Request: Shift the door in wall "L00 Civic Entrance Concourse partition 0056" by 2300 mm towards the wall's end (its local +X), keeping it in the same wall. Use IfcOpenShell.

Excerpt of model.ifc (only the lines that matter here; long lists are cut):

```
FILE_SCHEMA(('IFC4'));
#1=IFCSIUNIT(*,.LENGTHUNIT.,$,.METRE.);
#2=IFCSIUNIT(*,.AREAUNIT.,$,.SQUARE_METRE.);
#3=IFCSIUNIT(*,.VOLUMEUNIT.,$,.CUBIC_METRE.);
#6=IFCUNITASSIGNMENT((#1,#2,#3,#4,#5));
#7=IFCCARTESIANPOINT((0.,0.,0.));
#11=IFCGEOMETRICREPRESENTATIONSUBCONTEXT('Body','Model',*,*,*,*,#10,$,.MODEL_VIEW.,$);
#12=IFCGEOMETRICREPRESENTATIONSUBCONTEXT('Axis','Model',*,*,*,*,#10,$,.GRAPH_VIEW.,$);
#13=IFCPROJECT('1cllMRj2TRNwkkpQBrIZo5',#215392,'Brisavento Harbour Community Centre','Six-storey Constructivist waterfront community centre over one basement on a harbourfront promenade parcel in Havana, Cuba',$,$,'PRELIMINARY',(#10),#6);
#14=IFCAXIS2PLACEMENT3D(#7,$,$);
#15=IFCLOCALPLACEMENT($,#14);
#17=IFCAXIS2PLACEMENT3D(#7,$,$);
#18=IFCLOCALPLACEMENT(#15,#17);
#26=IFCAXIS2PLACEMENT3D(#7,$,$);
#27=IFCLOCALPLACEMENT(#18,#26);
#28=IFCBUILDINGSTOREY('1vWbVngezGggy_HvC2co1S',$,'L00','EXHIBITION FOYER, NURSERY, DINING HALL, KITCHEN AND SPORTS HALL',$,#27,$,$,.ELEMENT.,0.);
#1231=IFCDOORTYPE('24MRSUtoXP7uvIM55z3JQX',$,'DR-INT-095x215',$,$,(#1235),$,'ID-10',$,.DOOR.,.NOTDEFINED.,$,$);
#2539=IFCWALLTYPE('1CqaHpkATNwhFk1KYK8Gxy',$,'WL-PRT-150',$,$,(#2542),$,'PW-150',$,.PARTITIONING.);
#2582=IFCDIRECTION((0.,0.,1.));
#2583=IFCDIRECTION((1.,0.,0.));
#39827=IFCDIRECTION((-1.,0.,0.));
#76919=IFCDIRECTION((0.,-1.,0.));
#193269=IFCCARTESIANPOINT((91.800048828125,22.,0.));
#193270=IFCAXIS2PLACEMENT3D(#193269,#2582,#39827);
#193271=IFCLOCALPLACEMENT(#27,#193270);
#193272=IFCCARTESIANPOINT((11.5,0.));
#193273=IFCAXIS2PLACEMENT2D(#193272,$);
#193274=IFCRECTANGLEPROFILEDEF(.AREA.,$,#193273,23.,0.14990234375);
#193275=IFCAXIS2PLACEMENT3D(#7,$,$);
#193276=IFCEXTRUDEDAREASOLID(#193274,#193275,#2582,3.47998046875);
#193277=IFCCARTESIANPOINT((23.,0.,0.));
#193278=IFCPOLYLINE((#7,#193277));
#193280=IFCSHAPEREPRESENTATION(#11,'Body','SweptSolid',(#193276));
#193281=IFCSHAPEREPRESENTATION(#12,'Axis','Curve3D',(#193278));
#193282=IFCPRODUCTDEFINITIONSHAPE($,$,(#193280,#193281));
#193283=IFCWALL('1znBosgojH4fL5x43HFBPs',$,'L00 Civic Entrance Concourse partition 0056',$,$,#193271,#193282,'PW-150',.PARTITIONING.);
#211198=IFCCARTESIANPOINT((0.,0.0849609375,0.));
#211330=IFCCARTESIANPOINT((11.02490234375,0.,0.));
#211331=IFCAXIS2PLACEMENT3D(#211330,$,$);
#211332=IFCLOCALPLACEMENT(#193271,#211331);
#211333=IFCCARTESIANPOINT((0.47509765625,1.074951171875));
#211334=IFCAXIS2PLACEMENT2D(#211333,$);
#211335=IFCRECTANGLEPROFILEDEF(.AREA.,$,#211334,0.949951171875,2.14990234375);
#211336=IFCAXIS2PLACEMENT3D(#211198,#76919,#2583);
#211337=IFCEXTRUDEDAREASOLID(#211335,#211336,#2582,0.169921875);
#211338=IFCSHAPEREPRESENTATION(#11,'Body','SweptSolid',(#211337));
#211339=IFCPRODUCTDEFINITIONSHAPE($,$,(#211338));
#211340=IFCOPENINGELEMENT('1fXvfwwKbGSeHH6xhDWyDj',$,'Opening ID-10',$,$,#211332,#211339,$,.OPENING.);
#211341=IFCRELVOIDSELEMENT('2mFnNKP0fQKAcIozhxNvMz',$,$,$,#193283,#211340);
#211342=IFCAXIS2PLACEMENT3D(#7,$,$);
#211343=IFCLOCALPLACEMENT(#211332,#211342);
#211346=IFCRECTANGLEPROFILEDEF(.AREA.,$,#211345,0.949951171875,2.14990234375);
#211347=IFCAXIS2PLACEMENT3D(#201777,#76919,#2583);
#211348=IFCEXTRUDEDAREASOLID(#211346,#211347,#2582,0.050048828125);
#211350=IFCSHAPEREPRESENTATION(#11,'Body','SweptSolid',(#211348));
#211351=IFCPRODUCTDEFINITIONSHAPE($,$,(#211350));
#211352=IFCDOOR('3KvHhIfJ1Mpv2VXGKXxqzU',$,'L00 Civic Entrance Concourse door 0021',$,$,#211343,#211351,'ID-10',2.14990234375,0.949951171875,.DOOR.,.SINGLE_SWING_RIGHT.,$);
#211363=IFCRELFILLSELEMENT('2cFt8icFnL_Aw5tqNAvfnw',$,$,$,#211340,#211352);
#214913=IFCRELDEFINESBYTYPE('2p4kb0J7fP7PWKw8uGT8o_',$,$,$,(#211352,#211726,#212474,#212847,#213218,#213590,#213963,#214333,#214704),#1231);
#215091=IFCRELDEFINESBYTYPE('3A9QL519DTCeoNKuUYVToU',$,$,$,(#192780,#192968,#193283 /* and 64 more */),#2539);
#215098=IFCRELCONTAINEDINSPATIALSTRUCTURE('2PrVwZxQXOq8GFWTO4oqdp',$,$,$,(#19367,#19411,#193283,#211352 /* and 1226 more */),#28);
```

```python
import ifcopenshell
import ifcopenshell.api.geometry
import ifcopenshell.util.placement
import ifcopenshell.util.unit

model = ifcopenshell.open("model.ifc")
unit_scale = ifcopenshell.util.unit.calculate_unit_scale(model)

door = model.by_id(211352)
opening = door.FillsVoids[0].RelatingOpeningElement
wall = opening.VoidsElements[0].RelatingBuildingElement

wall_matrix = ifcopenshell.util.placement.get_local_placement(wall.ObjectPlacement)
shift = wall_matrix[:3, 0] * 2.3 / unit_scale
before = ifcopenshell.util.placement.get_local_placement(door.ObjectPlacement)[:3, 3].copy()

# The door is placed relative to its opening, so it follows when the opening moves.
matrix = ifcopenshell.util.placement.get_local_placement(opening.ObjectPlacement)
matrix[:3, 3] += shift
ifcopenshell.api.geometry.edit_object_placement(
    model, product=opening, matrix=matrix, is_si=False, should_transform_children=True
)

after = ifcopenshell.util.placement.get_local_placement(door.ObjectPlacement)[:3, 3]
print("door moved by", (after - before).round(3) + 0.0)

model.write("model_edited.ifc")
```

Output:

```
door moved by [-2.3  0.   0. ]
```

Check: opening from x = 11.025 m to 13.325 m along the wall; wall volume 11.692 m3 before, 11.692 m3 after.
